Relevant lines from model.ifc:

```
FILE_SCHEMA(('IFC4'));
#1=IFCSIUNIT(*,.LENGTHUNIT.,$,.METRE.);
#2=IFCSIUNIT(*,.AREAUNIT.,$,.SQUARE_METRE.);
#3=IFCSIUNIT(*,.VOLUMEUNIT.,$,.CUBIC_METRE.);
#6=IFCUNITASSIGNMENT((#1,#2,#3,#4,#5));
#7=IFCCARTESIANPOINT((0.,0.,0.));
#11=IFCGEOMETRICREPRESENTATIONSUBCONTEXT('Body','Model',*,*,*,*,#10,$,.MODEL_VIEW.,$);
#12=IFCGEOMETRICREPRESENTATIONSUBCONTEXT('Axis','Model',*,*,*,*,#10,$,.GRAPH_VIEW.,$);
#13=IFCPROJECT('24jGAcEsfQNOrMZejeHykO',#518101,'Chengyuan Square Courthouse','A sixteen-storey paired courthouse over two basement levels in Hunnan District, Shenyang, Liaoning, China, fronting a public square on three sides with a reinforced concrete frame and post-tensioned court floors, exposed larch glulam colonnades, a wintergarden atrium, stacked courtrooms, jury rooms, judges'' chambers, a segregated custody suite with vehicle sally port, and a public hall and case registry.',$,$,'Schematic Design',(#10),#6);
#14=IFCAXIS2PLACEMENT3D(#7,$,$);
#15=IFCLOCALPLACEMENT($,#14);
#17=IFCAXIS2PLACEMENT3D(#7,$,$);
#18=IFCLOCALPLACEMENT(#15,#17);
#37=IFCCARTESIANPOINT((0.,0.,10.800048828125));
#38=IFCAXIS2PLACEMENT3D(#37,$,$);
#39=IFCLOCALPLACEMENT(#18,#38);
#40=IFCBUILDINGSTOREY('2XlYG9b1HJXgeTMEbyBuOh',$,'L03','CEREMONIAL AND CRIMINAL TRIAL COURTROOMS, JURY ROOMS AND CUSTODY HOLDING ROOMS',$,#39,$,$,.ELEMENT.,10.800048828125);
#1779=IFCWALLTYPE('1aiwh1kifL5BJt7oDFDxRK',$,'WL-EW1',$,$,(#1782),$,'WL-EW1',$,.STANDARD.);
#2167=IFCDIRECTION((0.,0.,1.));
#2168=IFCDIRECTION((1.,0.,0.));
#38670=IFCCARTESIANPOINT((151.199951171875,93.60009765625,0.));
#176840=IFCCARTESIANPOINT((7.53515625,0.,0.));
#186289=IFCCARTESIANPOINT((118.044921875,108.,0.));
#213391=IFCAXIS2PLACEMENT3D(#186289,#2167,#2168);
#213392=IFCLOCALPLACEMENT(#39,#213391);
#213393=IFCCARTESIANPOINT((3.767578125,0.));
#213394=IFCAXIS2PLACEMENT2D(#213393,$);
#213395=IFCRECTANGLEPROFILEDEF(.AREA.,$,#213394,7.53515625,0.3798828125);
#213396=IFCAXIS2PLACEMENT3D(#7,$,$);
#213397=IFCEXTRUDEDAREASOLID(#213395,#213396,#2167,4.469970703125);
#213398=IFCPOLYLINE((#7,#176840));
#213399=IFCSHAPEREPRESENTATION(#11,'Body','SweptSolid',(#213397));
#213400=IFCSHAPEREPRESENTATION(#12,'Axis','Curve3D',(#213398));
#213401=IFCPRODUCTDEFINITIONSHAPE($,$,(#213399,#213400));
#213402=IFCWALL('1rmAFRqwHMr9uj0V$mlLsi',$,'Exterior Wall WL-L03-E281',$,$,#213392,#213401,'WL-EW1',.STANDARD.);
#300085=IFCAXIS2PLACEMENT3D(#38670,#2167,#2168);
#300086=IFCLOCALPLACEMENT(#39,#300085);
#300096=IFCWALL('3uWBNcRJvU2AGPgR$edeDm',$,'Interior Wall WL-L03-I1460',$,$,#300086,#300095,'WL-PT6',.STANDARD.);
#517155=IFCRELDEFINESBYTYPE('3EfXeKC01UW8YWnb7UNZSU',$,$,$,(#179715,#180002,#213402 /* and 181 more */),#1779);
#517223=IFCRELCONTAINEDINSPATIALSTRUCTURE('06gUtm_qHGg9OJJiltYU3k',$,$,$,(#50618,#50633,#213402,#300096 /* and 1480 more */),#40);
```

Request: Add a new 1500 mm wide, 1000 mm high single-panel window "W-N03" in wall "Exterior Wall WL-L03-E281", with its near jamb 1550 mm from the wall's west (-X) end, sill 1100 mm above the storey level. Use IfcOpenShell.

```python
import numpy as np
import ifcopenshell
import ifcopenshell.api.feature
import ifcopenshell.api.geometry
import ifcopenshell.api.root
import ifcopenshell.api.spatial
import ifcopenshell.geom
import ifcopenshell.util.element
import ifcopenshell.util.placement
import ifcopenshell.util.representation
import ifcopenshell.util.shape
import ifcopenshell.util.unit

model = ifcopenshell.open("model.ifc")
unit_scale = ifcopenshell.util.unit.calculate_unit_scale(model)
settings = ifcopenshell.geom.settings()


def volume(element):
    """Net volume in cubic metres, openings subtracted."""
    shape = ifcopenshell.geom.create_shape(settings, element)
    return ifcopenshell.util.shape.get_volume(shape.geometry)


wall = model.by_guid("1rmAFRqwHMr9uj0V$mlLsi")
storey = ifcopenshell.util.element.get_container(wall, ifc_class="IfcBuildingStorey")
context = ifcopenshell.util.representation.get_context(model, "Model", "Body", "MODEL_VIEW")
before = volume(wall)

width, height, from_end, sill = 1.5, 1, 1.55, 1.1  # metres

# The wall runs along its own X axis, and the end named is its -X end.
wall_shape = ifcopenshell.geom.create_shape(settings, wall)
x, y, z = ifcopenshell.util.shape.get_vertices(wall_shape.geometry).T
start = x.min() + from_end
face, thickness = float(y.min()), float(y.max() - y.min())
wall_matrix = ifcopenshell.util.placement.get_local_placement(wall.ObjectPlacement)
level = ifcopenshell.util.placement.get_local_placement(storey.ObjectPlacement)[2, 3]


def in_wall(x, y):
    """Placement at x, y metres in the wall's axes, at sill height."""
    matrix = wall_matrix.copy()
    matrix[:, 3] = wall_matrix @ np.array([x / unit_scale, y / unit_scale, 0.0, 1.0])
    matrix[2, 3] = level + sill / unit_scale
    return matrix


# Opening: a box that overshoots both wall faces by 50 mm.
opening = ifcopenshell.api.root.create_entity(model, ifc_class="IfcOpeningElement", predefined_type="OPENING")
box = ifcopenshell.api.geometry.add_wall_representation(
    model, context=context, length=width, height=height, thickness=thickness + 0.1
)
ifcopenshell.api.geometry.assign_representation(model, product=opening, representation=box)
ifcopenshell.api.geometry.edit_object_placement(model, product=opening, matrix=in_wall(start, face - 0.05), is_si=False)
ifcopenshell.api.feature.add_feature(model, feature=opening, element=wall)

window = ifcopenshell.api.root.create_entity(model, ifc_class="IfcWindow", name="W-N03", predefined_type="WINDOW")
window.OverallWidth, window.OverallHeight = width / unit_scale, height / unit_scale
window.PartitioningType = "SINGLE_PANEL"
body = ifcopenshell.api.geometry.add_window_representation(
    model,
    context=context,
    overall_width=window.OverallWidth,
    overall_height=window.OverallHeight,
    partition_type="SINGLE_PANEL",
)
ifcopenshell.api.geometry.assign_representation(model, product=window, representation=body)
ifcopenshell.api.spatial.assign_container(model, products=[window], relating_structure=storey)
ifcopenshell.api.feature.add_filling(model, opening=opening, element=window)

# Centre the window in the wall's thickness.
ifcopenshell.api.geometry.edit_object_placement(model, product=window, matrix=in_wall(start, face), is_si=False)
window_shape = ifcopenshell.geom.create_shape(settings, window)
depth = ifcopenshell.util.shape.get_vertices(window_shape.geometry)[:, 1]
offset = face + thickness / 2 - (depth.min() + depth.max()) / 2
ifcopenshell.api.geometry.edit_object_placement(model, product=window, matrix=in_wall(start, offset), is_si=False)

after = volume(wall)

print(f"wall volume {before:.3f} -> {after:.3f} m3")

model.write("model_v2.ifc")
```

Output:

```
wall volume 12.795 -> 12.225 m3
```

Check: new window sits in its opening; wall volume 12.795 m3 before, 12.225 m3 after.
